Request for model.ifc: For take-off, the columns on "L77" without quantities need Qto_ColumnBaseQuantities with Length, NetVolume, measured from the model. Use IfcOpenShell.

First a look at what the model holds.

```python
import ifcopenshell
import ifcopenshell.util.element
import ifcopenshell.util.unit

model = ifcopenshell.open("model.ifc")
print(model.schema)
for unit_type in ("LENGTHUNIT", "AREAUNIT", "VOLUMEUNIT"):
    print(unit_type, ifcopenshell.util.unit.calculate_unit_scale(model, unit_type))
storey = next(s for s in model.by_type("IfcBuildingStorey") if s.Name == "L77")
columns = [e for e in ifcopenshell.util.element.get_decomposition(storey) if e.is_a("IfcColumn")]
for e in sorted(columns, key=lambda e: e.id()):
    print(e.id(), e.is_a(), e.Name, list(ifcopenshell.util.element.get_psets(e, qtos_only=True)), sep=" | ")
```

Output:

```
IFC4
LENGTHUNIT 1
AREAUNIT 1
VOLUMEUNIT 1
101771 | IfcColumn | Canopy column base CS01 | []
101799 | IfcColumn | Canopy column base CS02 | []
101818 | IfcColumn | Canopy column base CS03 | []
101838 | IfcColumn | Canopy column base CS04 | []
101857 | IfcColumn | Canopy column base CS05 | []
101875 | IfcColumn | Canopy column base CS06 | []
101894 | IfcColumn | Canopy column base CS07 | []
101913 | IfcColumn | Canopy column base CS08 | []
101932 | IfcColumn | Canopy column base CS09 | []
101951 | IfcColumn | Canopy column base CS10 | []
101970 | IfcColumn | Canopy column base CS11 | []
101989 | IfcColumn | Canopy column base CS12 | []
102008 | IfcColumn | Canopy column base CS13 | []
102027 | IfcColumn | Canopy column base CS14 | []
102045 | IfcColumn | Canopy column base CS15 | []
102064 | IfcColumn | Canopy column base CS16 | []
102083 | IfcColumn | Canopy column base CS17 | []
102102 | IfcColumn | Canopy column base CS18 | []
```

```python
import ifcopenshell
import ifcopenshell.api.pset
import ifcopenshell.geom
import ifcopenshell.util.element
import ifcopenshell.util.shape
import ifcopenshell.util.unit

model = ifcopenshell.open("model.ifc")
unit_scale = ifcopenshell.util.unit.calculate_unit_scale(model)
volume_scale = ifcopenshell.util.unit.calculate_unit_scale(model, "VOLUMEUNIT")
settings = ifcopenshell.geom.settings()

storey = next(s for s in model.by_type("IfcBuildingStorey") if s.Name == "L77")
columns = [e for e in ifcopenshell.util.element.get_decomposition(storey) if e.is_a("IfcColumn")]

for e in sorted(columns, key=lambda e: e.id()):
    if ifcopenshell.util.element.get_psets(e, qtos_only=True, should_inherit=False):
        continue
    # Geometry comes back in metres, in the element's own axes.
    shape = ifcopenshell.geom.create_shape(settings, e)
    values = {
        "Length": ifcopenshell.util.shape.get_z(shape.geometry) / unit_scale,
        "NetVolume": ifcopenshell.util.shape.get_volume(shape.geometry) / volume_scale,
    }
    qto = ifcopenshell.api.pset.add_qto(model, product=e, name="Qto_ColumnBaseQuantities")
    ifcopenshell.api.pset.edit_qto(model, qto=qto, properties=values)
    print(e.id(), {k: round(v, 3) for k, v in values.items()})

model.write("model_updated.ifc")
```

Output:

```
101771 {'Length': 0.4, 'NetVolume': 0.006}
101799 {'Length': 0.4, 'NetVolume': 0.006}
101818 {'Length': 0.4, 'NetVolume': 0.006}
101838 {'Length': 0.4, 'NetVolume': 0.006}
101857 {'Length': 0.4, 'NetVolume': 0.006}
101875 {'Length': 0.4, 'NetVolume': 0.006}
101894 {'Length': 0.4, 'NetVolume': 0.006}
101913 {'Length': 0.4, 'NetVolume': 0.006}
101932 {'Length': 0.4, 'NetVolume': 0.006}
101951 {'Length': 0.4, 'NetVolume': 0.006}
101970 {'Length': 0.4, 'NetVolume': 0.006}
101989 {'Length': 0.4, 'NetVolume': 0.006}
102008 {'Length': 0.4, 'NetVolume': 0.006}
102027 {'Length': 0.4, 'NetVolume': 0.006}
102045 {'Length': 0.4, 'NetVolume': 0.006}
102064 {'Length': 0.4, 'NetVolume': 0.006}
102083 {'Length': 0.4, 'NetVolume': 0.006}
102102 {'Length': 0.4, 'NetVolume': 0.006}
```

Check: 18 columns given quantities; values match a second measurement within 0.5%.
